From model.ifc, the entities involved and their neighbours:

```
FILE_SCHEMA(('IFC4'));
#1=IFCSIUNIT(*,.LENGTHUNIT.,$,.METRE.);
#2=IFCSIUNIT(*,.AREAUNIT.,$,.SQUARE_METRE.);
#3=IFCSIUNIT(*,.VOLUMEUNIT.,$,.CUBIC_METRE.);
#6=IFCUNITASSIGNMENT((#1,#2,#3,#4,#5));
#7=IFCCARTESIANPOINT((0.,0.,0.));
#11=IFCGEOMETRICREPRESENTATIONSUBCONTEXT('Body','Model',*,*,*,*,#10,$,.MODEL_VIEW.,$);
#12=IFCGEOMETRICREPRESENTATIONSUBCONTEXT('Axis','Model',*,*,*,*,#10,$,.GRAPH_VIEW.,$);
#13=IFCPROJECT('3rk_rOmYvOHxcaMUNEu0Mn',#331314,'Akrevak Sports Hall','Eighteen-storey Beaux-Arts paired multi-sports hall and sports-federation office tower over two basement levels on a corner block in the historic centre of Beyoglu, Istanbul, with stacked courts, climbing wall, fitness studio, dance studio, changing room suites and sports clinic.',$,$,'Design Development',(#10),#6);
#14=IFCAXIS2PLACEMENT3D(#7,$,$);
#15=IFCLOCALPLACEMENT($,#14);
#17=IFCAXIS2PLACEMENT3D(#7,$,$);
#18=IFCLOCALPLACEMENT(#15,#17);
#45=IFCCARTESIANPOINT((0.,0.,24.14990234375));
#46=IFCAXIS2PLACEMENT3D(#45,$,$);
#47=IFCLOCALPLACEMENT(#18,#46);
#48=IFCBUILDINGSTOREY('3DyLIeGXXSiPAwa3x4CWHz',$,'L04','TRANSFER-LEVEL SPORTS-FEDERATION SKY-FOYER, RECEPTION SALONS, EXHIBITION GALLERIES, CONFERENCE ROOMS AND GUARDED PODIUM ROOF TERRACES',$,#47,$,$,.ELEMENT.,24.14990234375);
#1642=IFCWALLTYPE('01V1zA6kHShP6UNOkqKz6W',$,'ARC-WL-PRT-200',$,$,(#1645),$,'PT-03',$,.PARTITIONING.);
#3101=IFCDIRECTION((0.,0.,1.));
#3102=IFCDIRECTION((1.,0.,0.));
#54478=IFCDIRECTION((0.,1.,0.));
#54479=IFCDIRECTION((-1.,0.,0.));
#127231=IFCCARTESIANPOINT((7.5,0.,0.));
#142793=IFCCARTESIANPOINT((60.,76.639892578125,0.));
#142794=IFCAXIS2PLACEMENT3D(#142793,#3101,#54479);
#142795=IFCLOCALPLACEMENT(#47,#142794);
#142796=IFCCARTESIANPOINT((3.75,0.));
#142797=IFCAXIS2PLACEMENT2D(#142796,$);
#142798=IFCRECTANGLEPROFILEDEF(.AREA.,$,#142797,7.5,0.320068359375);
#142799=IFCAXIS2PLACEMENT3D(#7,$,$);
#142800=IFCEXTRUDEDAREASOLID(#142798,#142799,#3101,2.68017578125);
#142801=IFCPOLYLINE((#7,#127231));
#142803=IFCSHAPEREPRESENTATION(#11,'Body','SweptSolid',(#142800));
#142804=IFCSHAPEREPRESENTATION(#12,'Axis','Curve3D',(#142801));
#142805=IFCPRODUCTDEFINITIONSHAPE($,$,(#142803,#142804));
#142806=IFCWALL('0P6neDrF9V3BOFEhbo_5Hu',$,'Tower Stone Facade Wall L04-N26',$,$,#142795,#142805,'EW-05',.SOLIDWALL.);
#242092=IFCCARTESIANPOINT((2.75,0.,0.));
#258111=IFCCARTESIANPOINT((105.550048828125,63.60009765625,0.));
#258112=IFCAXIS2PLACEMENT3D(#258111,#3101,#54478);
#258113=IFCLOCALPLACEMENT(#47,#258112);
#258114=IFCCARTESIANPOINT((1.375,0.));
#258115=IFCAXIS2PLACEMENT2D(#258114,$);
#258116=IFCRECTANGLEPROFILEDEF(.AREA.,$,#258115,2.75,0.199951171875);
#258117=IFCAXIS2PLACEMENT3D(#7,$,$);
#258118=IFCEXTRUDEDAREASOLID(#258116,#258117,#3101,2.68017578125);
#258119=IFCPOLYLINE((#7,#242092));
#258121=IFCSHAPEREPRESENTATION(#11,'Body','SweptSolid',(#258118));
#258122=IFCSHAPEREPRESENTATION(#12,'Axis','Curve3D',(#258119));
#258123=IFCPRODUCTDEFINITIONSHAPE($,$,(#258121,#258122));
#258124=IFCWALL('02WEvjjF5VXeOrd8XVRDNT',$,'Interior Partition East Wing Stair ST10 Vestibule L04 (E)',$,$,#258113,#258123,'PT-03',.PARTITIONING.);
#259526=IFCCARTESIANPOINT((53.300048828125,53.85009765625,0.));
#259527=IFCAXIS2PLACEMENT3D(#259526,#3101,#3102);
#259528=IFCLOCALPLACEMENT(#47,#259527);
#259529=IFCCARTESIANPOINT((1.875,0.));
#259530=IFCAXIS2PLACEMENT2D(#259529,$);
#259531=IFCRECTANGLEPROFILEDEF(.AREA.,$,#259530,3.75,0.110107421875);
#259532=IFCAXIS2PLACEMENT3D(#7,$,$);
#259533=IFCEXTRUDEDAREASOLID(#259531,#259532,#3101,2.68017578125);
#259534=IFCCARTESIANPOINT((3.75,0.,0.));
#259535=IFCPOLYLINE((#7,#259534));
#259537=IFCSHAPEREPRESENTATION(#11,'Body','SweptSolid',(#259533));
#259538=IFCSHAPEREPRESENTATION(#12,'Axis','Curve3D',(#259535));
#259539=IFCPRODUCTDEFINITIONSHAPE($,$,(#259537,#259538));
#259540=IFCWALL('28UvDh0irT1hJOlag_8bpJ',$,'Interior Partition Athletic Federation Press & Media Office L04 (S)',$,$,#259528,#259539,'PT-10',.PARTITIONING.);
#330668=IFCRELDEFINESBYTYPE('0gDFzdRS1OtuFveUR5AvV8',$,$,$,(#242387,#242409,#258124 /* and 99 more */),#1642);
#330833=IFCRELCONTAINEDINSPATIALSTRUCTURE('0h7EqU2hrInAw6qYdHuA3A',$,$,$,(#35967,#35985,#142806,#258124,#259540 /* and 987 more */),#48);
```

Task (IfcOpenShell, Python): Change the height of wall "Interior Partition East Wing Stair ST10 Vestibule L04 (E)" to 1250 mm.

```python
import ifcopenshell
import ifcopenshell.geom
import ifcopenshell.util.representation
import ifcopenshell.util.shape
import ifcopenshell.util.unit

model = ifcopenshell.open("model.ifc")
unit_scale = ifcopenshell.util.unit.calculate_unit_scale(model)
settings = ifcopenshell.geom.settings()


def volume(element):
    """Net volume in cubic metres, openings subtracted."""
    shape = ifcopenshell.geom.create_shape(settings, element)
    return ifcopenshell.util.shape.get_volume(shape.geometry)


wall = model.by_guid("02WEvjjF5VXeOrd8XVRDNT")
before = volume(wall)

body = ifcopenshell.util.representation.get_representation(wall, "Model", "Body")
solid = body.Items[0]
old_height = solid.Depth
solid.Depth = 1.25 / unit_scale
after = volume(wall)

print(f"height {old_height:g} -> {solid.Depth:g}, volume {before:.3f} -> {after:.3f} m3")

model.write("model_edited.ifc")
```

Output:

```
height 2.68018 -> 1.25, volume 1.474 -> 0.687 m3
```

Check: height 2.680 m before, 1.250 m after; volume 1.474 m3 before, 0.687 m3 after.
